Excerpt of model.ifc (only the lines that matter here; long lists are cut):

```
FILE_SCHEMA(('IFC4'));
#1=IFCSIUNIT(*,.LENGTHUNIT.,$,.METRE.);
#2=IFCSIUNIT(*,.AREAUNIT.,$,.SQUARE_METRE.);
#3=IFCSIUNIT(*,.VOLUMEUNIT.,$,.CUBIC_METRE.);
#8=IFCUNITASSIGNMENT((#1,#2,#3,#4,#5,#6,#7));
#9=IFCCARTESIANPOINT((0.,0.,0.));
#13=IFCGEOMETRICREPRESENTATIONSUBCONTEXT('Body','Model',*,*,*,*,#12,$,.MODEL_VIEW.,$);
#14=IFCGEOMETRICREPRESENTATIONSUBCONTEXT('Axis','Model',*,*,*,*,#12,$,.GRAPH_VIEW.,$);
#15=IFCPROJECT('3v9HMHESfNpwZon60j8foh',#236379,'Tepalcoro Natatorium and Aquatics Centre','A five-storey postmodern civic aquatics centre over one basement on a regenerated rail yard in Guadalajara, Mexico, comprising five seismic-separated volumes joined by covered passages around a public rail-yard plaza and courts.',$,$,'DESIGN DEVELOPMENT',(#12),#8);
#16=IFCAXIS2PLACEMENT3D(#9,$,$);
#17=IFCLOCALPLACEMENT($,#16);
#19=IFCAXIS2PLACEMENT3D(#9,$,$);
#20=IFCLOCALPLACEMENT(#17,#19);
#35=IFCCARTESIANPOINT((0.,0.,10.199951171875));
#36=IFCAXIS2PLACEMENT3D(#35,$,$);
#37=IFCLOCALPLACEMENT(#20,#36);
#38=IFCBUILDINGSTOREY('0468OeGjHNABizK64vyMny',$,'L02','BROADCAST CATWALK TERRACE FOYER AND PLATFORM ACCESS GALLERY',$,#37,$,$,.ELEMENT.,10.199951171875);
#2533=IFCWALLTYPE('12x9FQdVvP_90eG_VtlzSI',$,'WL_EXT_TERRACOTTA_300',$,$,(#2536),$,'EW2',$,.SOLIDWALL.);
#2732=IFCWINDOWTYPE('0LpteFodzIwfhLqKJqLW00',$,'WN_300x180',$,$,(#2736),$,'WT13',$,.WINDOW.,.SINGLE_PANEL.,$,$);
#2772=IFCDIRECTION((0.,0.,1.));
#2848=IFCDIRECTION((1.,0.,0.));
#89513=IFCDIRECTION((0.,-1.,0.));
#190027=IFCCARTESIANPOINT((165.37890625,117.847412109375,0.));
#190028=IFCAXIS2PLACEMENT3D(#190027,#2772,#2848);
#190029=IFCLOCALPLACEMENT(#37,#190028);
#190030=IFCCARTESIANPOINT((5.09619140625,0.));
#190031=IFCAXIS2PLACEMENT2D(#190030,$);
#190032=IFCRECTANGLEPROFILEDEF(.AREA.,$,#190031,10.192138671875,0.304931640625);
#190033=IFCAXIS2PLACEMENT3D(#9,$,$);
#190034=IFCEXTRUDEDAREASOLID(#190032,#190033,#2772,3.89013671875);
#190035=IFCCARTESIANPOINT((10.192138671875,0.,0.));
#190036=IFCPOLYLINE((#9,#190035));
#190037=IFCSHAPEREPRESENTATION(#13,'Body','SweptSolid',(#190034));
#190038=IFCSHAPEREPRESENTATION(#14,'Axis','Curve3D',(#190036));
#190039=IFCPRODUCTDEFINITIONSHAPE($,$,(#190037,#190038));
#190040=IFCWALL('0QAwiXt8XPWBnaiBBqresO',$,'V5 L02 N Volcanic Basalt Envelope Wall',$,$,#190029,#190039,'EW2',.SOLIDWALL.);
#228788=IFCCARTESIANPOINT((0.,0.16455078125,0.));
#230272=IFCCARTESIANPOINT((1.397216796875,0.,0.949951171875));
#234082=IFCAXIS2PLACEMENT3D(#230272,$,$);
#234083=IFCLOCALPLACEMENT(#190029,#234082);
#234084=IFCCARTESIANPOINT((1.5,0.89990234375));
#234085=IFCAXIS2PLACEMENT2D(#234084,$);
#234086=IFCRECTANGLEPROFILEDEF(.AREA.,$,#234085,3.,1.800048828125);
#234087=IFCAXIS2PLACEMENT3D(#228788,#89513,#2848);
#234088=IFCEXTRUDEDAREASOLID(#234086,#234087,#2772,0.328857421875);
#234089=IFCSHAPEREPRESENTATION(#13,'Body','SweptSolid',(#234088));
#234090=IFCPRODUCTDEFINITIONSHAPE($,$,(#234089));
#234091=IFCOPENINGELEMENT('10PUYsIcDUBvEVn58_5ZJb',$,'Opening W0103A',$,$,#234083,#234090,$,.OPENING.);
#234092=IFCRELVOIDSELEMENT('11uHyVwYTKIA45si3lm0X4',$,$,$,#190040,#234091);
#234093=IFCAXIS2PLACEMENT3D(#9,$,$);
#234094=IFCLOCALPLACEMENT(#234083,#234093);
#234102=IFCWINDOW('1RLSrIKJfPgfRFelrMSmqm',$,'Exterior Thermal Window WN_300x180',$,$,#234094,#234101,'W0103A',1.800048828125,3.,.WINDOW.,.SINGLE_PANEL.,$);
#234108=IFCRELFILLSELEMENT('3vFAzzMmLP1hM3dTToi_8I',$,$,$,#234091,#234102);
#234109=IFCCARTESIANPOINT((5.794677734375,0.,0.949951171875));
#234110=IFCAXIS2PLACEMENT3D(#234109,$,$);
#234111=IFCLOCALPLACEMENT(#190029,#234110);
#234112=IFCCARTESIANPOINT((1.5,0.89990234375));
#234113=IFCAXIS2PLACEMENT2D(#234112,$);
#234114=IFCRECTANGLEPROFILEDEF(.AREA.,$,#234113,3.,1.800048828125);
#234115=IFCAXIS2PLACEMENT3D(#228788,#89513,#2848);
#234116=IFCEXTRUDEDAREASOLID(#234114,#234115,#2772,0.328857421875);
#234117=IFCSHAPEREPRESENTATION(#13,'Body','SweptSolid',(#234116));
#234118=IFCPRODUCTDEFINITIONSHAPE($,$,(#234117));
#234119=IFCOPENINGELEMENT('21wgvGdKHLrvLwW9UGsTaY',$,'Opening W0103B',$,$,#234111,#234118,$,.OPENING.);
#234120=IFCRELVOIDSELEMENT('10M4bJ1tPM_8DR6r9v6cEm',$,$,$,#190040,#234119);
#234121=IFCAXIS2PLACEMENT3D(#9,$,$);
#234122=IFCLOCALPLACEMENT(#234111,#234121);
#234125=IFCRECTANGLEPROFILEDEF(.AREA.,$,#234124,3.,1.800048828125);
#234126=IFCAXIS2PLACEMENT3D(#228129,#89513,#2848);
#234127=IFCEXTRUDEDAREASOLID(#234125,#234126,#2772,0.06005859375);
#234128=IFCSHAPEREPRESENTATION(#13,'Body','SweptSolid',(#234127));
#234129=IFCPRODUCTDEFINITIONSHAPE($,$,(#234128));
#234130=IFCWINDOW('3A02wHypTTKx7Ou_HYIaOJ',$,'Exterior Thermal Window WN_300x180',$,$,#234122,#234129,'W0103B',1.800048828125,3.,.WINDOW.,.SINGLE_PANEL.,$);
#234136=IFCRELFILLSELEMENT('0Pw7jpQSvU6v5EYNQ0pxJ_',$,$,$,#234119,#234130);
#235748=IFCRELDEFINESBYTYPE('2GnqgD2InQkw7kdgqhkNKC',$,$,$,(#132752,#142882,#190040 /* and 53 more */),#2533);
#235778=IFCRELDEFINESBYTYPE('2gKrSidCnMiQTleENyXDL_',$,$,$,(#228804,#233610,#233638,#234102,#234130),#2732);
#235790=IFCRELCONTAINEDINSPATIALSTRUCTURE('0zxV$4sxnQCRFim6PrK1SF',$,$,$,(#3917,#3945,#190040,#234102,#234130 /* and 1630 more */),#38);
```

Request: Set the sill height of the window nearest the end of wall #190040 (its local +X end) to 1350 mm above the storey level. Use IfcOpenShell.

```python
import numpy as np
import ifcopenshell
import ifcopenshell.api.geometry
import ifcopenshell.geom
import ifcopenshell.util.element
import ifcopenshell.util.placement
import ifcopenshell.util.shape
import ifcopenshell.util.unit

model = ifcopenshell.open("model.ifc")
unit_scale = ifcopenshell.util.unit.calculate_unit_scale(model)

window = model.by_guid("3A02wHypTTKx7Ou_HYIaOJ")
opening = window.FillsVoids[0].RelatingOpeningElement
storey = ifcopenshell.util.element.get_container(window, ifc_class="IfcBuildingStorey")
level = ifcopenshell.util.placement.get_local_placement(storey.ObjectPlacement)[2, 3]

# The opening's origin need not be at the sill, so measure its lowest point.
shape = ifcopenshell.geom.create_shape(ifcopenshell.geom.settings(), opening)
bottom = ifcopenshell.util.shape.get_shape_bottom_elevation(shape, shape.geometry) / unit_scale
dz = level + 1.35 / unit_scale - bottom

shift = np.array([0.0, 0.0, dz])
# The window is placed relative to its opening, so it follows when the opening moves.
matrix = ifcopenshell.util.placement.get_local_placement(opening.ObjectPlacement)
matrix[:3, 3] += shift
ifcopenshell.api.geometry.edit_object_placement(
    model, product=opening, matrix=matrix, is_si=False, should_transform_children=True
)

print(f"moved by {dz * unit_scale:+.3f} m")

model.write("model_rev.ifc")
```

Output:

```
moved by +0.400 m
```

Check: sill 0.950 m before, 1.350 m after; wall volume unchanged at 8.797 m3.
